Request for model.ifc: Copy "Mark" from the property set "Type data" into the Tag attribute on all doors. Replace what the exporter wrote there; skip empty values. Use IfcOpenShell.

First a look at what the model holds.

```python
import ifcopenshell
import ifcopenshell.util.element

model = ifcopenshell.open("model.ifc")
print(model.schema)
doors = model.by_type("IfcDoor")
print(len(doors), "doors")
for e in doors[:8]:
    source = ifcopenshell.util.element.get_pset(e, "Type data", "Mark")
    target = e.Tag
    print(e.id(), repr(source), repr(target), sep=" | ")
```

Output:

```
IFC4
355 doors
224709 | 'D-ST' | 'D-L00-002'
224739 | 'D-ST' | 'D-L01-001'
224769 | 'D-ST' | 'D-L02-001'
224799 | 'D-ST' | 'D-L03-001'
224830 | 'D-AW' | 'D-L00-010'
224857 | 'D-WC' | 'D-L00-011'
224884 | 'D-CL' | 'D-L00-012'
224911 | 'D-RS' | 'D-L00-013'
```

```python
import ifcopenshell
import ifcopenshell.util.element

model = ifcopenshell.open("model.ifc")

count = 0
for e in model.by_type("IfcDoor"):
    value = ifcopenshell.util.element.get_pset(e, "Type data", "Mark")
    current = e.Tag
    if not value or not value.strip() or current == value:
        continue
    e.Tag = value
    count += 1

print(count, "doors updated")

model.write("model_updated.ifc")
```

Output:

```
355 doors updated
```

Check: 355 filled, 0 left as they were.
